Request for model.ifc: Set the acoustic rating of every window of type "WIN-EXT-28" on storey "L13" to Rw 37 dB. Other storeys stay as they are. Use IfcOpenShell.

First a look at what the model holds.

```python
import ifcopenshell
import ifcopenshell.util.element

model = ifcopenshell.open("model.ifc")
print(model.schema)
storey = next(s for s in model.by_type("IfcBuildingStorey") if s.Name == "L13")
windows = [e for e in ifcopenshell.util.element.get_decomposition(storey) if e.is_a("IfcWindow")]
seen = {}
for e in windows:
    element_type = ifcopenshell.util.element.get_type(e)
    key = (element_type.Name if element_type != e and element_type else None, ifcopenshell.util.element.get_pset(e, "Pset_WindowCommon", "AcousticRating"))
    seen[key] = seen.get(key, 0) + 1
for (name, value), count in sorted(seen.items(), key=str):
    print(count, "x", name, "|", value)
```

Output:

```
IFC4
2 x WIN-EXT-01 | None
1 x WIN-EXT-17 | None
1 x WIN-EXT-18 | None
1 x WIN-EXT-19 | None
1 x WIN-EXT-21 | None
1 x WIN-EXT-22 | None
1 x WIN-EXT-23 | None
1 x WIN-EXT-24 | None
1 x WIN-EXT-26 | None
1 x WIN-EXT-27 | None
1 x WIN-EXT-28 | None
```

```python
import ifcopenshell
import ifcopenshell.api.pset
import ifcopenshell.util.element

model = ifcopenshell.open("model.ifc")

storey = next(s for s in model.by_type("IfcBuildingStorey") if s.Name == "L13")
windows = [e for e in ifcopenshell.util.element.get_decomposition(storey) if e.is_a("IfcWindow")]

count = 0
for e in windows:
    element_type = ifcopenshell.util.element.get_type(e)
    if element_type in (None, e) or element_type.Name != "WIN-EXT-28":
        continue
    # add_pset returns the element's existing set when there is one.
    pset = ifcopenshell.api.pset.add_pset(model, product=e, name="Pset_WindowCommon")
    ifcopenshell.api.pset.edit_pset(model, pset=pset, properties={"AcousticRating": "Rw 37 dB"})
    count += 1

print(count, "windows updated")

model.write("model_edited.ifc")
```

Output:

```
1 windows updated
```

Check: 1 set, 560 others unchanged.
